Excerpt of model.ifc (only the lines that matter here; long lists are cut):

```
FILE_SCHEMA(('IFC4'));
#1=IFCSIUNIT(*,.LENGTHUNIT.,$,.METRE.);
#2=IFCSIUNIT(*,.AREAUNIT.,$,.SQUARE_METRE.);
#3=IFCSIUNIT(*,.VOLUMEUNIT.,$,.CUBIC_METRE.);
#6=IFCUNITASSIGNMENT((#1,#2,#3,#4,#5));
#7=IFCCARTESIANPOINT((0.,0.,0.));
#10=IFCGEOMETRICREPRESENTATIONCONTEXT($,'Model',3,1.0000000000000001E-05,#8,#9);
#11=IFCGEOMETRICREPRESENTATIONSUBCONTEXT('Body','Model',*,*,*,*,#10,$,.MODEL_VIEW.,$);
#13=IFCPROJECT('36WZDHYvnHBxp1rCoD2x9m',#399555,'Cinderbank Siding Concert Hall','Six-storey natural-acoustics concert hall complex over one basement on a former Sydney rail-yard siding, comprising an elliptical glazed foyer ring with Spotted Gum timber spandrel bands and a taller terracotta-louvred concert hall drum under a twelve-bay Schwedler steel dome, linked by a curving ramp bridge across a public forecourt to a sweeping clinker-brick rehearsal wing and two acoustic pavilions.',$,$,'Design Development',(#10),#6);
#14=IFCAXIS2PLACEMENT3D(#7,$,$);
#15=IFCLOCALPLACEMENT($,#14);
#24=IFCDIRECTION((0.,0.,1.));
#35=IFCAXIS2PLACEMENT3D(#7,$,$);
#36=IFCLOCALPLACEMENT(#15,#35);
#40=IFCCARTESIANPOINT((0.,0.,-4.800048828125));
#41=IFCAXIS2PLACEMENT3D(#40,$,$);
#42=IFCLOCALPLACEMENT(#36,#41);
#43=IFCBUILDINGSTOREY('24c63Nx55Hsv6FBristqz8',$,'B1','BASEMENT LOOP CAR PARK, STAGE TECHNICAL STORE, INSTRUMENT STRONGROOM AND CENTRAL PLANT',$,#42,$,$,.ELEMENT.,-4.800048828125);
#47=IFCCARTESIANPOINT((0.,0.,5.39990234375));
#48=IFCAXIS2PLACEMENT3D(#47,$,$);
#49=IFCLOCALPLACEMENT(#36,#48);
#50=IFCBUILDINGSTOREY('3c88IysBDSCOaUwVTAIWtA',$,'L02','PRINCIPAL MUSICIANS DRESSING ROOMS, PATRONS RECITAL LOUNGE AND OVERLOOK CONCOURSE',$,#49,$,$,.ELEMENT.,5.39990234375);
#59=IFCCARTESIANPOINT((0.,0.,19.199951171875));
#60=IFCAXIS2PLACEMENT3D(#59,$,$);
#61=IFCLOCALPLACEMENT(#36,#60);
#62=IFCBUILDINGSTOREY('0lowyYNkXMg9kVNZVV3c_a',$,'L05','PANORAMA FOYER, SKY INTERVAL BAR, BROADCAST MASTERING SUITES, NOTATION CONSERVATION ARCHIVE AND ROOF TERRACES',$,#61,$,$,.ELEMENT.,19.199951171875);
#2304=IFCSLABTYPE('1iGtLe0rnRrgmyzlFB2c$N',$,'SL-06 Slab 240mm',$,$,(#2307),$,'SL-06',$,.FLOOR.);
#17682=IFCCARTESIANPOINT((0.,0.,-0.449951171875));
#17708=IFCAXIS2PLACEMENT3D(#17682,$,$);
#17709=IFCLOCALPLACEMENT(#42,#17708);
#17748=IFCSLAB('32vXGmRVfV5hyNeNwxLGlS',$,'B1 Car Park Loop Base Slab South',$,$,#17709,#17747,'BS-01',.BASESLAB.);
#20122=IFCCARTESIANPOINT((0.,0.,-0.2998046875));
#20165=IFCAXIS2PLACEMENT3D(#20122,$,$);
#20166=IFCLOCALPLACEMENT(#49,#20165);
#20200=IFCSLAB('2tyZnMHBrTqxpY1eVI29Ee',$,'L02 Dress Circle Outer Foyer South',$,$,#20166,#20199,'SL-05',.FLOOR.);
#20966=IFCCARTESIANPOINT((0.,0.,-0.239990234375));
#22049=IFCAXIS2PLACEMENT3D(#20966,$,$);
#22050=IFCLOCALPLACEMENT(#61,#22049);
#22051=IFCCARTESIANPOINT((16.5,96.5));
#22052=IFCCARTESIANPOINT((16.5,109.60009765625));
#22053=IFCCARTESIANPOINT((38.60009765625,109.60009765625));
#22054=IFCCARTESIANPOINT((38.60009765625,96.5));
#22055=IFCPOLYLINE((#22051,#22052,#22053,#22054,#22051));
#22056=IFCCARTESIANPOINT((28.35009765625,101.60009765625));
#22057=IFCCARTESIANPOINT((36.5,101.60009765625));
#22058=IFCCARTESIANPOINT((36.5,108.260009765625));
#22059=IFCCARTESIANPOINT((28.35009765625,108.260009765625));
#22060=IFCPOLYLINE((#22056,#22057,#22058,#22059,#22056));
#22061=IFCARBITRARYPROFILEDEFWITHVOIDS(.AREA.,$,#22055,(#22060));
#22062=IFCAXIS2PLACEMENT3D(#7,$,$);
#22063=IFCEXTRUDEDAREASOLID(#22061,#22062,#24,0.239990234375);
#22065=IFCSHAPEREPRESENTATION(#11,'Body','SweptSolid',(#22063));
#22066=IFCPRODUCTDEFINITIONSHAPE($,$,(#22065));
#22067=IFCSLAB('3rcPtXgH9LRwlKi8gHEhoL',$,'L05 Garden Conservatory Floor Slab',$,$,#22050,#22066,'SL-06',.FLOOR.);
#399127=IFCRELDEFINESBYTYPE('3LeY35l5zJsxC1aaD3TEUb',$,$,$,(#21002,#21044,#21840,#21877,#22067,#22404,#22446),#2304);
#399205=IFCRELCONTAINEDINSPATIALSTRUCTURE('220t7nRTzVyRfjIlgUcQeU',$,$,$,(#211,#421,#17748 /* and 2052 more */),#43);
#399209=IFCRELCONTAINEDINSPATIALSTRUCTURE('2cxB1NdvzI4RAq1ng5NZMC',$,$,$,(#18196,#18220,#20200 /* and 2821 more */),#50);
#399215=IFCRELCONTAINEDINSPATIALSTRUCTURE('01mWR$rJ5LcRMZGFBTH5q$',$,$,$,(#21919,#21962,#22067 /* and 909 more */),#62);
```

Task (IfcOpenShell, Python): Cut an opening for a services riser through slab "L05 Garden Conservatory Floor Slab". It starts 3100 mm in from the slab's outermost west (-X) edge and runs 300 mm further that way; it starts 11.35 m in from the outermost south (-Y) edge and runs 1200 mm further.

```python
import numpy as np
import ifcopenshell
import ifcopenshell.api.feature
import ifcopenshell.api.geometry
import ifcopenshell.api.root
import ifcopenshell.geom
import ifcopenshell.util.placement
import ifcopenshell.util.representation
import ifcopenshell.util.shape
import ifcopenshell.util.unit

model = ifcopenshell.open("model.ifc")
unit_scale = ifcopenshell.util.unit.calculate_unit_scale(model)
settings = ifcopenshell.geom.settings()


def volume(element):
    """Net volume in cubic metres, openings subtracted."""
    shape = ifcopenshell.geom.create_shape(settings, element)
    return ifcopenshell.util.shape.get_volume(shape.geometry)


slab = model.by_id(22067)
before = volume(slab)

# Extent in the slab's own axes, in metres. The edges named are its -X and -Y sides.
slab_shape = ifcopenshell.geom.create_shape(settings, slab)
vertices = ifcopenshell.util.shape.get_vertices(slab_shape.geometry)
x_min, y_min, bottom = vertices.min(axis=0)
top = vertices[:, 2].max()

opening = ifcopenshell.api.root.create_entity(model, ifc_class="IfcOpeningElement", name="Services riser opening", predefined_type="OPENING")
context = ifcopenshell.util.representation.get_context(model, "Model", "Body", "MODEL_VIEW")
width, depth = 0.3, 1.2
outline = [(0.0, 0.0), (width, 0.0), (width, depth), (0.0, depth), (0.0, 0.0)]
# Overshoot both faces by 50 mm so the cut is clean.
shape = ifcopenshell.api.geometry.add_slab_representation(
    model, context=context, depth=top - bottom + 0.1, polyline=outline
)
ifcopenshell.api.geometry.assign_representation(model, product=opening, representation=shape)

matrix = ifcopenshell.util.placement.get_local_placement(slab.ObjectPlacement)
matrix[:, 3] = matrix @ np.append(np.array([x_min + 3.1, y_min + 11.35, bottom - 0.05]) / unit_scale, 1.0)
ifcopenshell.api.geometry.edit_object_placement(model, product=opening, matrix=matrix, is_si=False)
ifcopenshell.api.feature.add_feature(model, feature=opening, element=slab)

after = volume(slab)

print(f"slab volume {before:.3f} -> {after:.3f} m3")

model.write("model_updated.ifc")
```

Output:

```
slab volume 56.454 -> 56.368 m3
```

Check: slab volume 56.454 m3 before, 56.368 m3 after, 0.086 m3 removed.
